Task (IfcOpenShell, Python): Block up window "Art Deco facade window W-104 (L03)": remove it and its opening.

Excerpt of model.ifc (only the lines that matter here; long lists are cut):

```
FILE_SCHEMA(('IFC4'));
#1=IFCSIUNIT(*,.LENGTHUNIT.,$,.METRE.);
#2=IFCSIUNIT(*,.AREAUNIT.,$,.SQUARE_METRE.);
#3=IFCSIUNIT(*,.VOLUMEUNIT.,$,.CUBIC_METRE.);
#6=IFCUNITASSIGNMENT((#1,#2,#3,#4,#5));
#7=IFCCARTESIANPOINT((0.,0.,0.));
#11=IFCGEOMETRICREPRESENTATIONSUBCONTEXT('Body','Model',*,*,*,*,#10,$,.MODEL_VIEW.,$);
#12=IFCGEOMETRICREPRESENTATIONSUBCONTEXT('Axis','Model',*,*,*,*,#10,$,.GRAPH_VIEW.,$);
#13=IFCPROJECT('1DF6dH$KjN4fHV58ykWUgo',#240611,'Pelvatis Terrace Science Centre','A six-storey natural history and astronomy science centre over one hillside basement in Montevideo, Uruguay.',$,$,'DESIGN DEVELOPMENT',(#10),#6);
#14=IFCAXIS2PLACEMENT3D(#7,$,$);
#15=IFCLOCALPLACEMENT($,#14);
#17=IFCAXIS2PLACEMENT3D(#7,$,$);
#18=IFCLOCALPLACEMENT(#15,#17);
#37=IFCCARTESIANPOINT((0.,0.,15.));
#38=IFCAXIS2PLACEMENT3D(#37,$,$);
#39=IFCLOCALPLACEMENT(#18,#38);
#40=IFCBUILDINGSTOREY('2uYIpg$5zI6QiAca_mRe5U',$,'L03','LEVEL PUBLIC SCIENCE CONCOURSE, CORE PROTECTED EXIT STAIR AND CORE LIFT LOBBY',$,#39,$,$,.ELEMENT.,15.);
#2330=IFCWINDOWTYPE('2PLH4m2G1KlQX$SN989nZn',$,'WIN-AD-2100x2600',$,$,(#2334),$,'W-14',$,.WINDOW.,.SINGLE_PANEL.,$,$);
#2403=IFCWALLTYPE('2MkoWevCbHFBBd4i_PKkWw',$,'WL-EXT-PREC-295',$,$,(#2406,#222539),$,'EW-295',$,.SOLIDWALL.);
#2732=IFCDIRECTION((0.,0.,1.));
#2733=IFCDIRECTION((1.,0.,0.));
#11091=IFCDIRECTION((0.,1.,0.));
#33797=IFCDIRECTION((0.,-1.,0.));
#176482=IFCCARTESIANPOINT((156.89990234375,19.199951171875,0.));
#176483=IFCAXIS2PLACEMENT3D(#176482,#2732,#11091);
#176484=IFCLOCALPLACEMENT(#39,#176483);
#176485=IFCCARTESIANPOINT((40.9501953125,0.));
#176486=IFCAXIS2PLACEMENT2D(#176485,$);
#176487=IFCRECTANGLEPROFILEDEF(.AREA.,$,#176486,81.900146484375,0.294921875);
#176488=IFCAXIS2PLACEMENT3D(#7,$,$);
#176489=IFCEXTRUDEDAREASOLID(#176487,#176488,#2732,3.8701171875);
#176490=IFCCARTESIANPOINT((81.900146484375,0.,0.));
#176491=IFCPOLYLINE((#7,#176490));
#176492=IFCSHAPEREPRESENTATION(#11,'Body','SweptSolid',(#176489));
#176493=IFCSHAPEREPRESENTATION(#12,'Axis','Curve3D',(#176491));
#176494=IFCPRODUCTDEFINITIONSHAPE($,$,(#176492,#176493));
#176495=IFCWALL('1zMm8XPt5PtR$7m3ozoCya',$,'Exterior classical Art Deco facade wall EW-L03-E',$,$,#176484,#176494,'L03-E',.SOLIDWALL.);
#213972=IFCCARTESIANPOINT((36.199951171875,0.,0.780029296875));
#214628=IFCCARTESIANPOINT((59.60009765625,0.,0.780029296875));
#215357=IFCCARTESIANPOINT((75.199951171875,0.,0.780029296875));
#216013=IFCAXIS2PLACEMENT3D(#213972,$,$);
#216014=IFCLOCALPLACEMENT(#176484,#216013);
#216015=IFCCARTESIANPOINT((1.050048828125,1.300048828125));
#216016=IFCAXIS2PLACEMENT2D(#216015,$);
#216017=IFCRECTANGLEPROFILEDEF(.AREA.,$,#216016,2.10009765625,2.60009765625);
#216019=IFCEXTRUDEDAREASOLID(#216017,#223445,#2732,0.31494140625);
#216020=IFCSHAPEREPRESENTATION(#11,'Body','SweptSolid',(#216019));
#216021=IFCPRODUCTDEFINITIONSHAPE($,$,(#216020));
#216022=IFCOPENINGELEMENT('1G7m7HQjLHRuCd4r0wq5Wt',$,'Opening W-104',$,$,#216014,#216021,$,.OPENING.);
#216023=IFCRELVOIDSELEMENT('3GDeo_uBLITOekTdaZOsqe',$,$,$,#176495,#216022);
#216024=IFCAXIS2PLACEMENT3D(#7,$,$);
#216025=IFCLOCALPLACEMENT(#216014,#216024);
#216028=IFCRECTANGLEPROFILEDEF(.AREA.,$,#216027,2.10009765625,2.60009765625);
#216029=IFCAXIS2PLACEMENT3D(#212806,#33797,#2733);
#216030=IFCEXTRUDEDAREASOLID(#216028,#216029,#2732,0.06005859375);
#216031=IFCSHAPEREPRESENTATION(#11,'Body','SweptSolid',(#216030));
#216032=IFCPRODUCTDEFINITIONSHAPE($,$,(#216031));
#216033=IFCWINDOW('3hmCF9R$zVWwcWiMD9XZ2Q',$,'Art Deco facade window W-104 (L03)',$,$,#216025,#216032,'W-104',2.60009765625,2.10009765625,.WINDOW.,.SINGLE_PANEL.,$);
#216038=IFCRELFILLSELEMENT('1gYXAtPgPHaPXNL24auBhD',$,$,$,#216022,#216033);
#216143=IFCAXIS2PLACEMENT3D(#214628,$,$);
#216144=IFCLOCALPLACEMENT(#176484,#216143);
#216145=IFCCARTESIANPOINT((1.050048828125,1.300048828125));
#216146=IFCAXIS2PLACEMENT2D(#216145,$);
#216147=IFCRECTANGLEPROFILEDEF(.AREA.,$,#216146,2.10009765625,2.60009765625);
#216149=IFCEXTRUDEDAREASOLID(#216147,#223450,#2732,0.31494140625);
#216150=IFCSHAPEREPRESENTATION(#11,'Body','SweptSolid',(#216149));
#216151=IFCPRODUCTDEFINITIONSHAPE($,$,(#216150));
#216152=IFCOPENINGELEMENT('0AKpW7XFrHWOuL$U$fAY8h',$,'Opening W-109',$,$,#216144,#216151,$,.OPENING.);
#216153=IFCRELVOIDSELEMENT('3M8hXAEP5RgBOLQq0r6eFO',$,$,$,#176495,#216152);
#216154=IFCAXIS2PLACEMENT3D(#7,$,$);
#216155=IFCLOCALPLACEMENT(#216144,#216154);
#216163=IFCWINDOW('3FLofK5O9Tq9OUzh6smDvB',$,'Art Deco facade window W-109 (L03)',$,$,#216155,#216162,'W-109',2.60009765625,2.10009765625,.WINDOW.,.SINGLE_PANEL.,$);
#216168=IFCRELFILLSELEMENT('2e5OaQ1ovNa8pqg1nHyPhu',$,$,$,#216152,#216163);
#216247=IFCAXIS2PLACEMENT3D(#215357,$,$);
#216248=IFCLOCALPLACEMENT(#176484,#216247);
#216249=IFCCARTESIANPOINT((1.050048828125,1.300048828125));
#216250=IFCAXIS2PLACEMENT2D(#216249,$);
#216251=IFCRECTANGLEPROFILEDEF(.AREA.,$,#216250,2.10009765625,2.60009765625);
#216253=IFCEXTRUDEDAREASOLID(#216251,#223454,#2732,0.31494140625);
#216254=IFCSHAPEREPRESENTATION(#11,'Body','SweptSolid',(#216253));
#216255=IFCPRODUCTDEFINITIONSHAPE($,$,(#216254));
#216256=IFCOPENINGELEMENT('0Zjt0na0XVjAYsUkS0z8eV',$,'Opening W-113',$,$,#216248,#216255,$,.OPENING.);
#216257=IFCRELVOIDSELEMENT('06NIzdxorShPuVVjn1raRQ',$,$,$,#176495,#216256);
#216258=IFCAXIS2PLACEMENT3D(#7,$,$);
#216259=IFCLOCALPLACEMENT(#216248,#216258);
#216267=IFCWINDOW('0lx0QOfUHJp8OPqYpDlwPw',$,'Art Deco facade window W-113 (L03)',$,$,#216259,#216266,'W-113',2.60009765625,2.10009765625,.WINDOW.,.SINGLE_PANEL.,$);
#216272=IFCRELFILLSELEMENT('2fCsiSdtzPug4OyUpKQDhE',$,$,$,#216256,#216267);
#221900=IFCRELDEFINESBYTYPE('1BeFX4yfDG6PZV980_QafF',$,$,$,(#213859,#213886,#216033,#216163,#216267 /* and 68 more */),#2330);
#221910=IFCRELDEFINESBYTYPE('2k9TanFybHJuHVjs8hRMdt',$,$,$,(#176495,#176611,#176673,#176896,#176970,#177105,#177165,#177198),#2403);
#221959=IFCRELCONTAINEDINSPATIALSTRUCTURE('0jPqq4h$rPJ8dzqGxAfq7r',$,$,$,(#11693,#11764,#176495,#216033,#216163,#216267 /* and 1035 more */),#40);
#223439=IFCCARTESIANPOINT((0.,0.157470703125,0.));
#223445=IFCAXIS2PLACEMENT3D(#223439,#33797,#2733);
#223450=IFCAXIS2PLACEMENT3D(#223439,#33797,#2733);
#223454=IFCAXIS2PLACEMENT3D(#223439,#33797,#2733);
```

```python
import ifcopenshell
import ifcopenshell.api.feature
import ifcopenshell.api.root
import ifcopenshell.geom
import ifcopenshell.util.shape

model = ifcopenshell.open("model.ifc")
settings = ifcopenshell.geom.settings()


def volume(element):
    """Net volume in cubic metres, openings subtracted."""
    shape = ifcopenshell.geom.create_shape(settings, element)
    return ifcopenshell.util.shape.get_volume(shape.geometry)


window = model.by_guid("3hmCF9R$zVWwcWiMD9XZ2Q")
opening = window.FillsVoids[0].RelatingOpeningElement
wall = opening.VoidsElements[0].RelatingBuildingElement
before = volume(wall)

ifcopenshell.api.root.remove_product(model, product=window)
ifcopenshell.api.feature.remove_feature(model, feature=opening)

after = volume(wall)

print(f"wall volume {before:.3f} -> {after:.3f} m3")

model.write("model_edited.ifc")
```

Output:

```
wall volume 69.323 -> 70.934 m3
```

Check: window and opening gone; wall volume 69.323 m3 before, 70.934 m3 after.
